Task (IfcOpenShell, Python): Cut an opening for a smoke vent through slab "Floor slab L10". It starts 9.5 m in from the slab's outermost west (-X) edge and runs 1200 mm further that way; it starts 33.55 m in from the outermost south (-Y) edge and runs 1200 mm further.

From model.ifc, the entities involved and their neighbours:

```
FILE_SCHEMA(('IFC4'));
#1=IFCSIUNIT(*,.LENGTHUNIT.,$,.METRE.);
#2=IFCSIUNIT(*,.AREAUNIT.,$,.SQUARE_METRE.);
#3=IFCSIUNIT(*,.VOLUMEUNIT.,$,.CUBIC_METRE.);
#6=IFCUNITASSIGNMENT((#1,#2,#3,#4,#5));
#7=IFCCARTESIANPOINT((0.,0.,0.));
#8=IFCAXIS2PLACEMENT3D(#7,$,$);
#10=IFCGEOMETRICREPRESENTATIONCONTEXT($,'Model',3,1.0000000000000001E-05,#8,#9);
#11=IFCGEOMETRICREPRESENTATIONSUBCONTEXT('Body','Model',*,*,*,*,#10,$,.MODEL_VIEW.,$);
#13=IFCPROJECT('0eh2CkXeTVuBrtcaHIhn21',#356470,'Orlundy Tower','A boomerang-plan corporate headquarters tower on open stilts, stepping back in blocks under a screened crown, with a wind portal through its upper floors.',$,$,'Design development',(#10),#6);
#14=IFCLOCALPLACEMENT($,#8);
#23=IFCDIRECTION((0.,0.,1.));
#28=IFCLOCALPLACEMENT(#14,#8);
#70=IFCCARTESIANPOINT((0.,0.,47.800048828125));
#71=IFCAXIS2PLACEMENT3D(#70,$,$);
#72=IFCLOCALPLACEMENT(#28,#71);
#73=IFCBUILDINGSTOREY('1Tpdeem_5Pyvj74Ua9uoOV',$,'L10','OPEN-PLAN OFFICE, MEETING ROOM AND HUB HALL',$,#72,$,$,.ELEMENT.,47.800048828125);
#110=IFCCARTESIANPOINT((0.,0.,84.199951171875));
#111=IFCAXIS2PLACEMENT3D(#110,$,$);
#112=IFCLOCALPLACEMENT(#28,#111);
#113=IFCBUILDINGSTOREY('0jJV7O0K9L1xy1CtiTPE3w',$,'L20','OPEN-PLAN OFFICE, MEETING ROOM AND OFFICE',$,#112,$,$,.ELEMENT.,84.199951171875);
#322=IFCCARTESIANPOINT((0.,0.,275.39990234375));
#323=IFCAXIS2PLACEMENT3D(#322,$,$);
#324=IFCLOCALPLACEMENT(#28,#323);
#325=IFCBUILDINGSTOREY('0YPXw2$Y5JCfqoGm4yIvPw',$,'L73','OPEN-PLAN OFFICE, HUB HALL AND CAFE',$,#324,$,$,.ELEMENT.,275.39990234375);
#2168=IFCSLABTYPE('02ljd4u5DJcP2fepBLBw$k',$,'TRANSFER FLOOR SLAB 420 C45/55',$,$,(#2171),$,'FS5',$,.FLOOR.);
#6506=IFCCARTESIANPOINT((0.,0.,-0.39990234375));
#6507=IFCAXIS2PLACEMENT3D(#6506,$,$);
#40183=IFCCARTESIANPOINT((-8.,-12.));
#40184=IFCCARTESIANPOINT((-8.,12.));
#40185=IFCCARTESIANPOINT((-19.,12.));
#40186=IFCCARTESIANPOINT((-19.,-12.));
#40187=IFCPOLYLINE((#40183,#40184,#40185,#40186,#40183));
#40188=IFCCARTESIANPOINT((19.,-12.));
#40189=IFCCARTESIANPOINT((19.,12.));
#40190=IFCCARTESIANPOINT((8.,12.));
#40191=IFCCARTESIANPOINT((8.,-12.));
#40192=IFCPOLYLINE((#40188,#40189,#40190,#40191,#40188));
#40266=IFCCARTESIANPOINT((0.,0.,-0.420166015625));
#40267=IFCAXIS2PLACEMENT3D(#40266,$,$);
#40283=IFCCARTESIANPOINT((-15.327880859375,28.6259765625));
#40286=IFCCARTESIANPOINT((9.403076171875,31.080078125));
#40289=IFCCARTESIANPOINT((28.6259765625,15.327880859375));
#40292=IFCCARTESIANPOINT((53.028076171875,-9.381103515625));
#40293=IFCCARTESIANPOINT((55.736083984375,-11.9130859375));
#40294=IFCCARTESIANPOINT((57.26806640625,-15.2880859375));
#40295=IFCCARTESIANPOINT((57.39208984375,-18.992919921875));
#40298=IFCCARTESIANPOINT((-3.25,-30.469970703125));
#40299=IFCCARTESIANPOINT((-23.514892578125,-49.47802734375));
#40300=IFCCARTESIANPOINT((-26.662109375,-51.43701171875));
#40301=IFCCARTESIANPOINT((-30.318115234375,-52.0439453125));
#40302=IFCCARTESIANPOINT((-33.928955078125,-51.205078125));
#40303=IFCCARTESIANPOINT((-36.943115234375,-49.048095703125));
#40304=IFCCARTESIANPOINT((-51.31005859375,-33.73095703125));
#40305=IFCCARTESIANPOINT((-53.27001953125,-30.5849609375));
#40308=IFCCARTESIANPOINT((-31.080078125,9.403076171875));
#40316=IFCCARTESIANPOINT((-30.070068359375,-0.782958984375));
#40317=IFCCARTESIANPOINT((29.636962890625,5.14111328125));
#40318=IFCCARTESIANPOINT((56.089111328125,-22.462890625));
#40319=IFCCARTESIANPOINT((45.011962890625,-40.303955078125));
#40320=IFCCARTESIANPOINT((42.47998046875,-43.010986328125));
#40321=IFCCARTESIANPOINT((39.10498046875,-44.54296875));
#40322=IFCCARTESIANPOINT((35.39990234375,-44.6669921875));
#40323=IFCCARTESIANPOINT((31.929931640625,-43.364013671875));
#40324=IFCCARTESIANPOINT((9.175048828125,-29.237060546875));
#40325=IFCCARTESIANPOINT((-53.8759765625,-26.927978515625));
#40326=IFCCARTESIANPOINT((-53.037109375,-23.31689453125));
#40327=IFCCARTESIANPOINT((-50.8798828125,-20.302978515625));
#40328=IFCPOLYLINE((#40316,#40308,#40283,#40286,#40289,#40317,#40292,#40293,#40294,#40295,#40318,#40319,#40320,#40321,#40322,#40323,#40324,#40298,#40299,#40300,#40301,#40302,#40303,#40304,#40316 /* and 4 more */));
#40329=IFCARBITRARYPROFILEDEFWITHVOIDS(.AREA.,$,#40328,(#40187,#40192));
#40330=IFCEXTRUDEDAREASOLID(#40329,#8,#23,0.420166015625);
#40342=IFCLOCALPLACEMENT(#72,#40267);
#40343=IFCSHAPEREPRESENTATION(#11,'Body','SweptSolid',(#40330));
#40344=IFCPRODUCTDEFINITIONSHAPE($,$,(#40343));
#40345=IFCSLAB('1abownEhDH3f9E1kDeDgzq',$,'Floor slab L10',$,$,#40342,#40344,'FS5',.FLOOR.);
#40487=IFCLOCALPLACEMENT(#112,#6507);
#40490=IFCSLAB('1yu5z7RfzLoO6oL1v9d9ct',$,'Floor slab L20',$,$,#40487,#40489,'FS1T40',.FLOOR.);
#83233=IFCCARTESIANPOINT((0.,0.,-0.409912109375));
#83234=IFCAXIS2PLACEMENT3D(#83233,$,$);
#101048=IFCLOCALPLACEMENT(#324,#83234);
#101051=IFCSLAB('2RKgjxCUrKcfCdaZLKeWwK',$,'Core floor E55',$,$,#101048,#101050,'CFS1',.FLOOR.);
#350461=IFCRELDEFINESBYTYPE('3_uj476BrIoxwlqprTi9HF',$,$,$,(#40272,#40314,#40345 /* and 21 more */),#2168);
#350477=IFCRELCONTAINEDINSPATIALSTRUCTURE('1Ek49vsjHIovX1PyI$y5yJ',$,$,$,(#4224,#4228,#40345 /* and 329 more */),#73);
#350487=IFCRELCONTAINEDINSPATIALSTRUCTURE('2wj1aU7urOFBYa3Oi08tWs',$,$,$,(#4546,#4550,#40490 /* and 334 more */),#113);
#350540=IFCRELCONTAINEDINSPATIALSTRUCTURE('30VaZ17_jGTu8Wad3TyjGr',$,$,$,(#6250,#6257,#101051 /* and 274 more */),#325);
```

```python
import numpy as np
import ifcopenshell
import ifcopenshell.api.feature
import ifcopenshell.api.geometry
import ifcopenshell.api.root
import ifcopenshell.geom
import ifcopenshell.util.placement
import ifcopenshell.util.representation
import ifcopenshell.util.shape
import ifcopenshell.util.unit

model = ifcopenshell.open("model.ifc")
unit_scale = ifcopenshell.util.unit.calculate_unit_scale(model)
settings = ifcopenshell.geom.settings()


def volume(element):
    """Net volume in cubic metres, openings subtracted."""
    shape = ifcopenshell.geom.create_shape(settings, element)
    return ifcopenshell.util.shape.get_volume(shape.geometry)


slab = model.by_id(40345)
before = volume(slab)

# Extent in the slab's own axes, in metres. The edges named are its -X and -Y sides.
slab_shape = ifcopenshell.geom.create_shape(settings, slab)
vertices = ifcopenshell.util.shape.get_vertices(slab_shape.geometry)
x_min, y_min, bottom = vertices.min(axis=0)
top = vertices[:, 2].max()

opening = ifcopenshell.api.root.create_entity(model, ifc_class="IfcOpeningElement", name="Smoke vent opening", predefined_type="OPENING")
context = ifcopenshell.util.representation.get_context(model, "Model", "Body", "MODEL_VIEW")
width, depth = 1.2, 1.2
outline = [(0.0, 0.0), (width, 0.0), (width, depth), (0.0, depth), (0.0, 0.0)]
# Overshoot both faces by 50 mm so the cut is clean.
shape = ifcopenshell.api.geometry.add_slab_representation(
    model, context=context, depth=top - bottom + 0.1, polyline=outline
)
ifcopenshell.api.geometry.assign_representation(model, product=opening, representation=shape)

matrix = ifcopenshell.util.placement.get_local_placement(slab.ObjectPlacement)
matrix[:, 3] = matrix @ np.append(np.array([x_min + 9.5, y_min + 33.55, bottom - 0.05]) / unit_scale, 1.0)
ifcopenshell.api.geometry.edit_object_placement(model, product=opening, matrix=matrix, is_si=False)
ifcopenshell.api.feature.add_feature(model, feature=opening, element=slab)

after = volume(slab)

print(f"slab volume {before:.3f} -> {after:.3f} m3")

model.write("model_updated.ifc")
```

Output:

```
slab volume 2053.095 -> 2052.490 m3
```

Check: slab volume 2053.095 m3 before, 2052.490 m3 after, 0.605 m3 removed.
